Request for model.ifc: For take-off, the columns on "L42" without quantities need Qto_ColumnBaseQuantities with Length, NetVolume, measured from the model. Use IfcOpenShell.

First a look at what the model holds.

```python
import ifcopenshell
import ifcopenshell.util.element
import ifcopenshell.util.unit

model = ifcopenshell.open("model.ifc")
print(model.schema)
for unit_type in ("LENGTHUNIT", "AREAUNIT", "VOLUMEUNIT"):
    print(unit_type, ifcopenshell.util.unit.calculate_unit_scale(model, unit_type))
storey = next(s for s in model.by_type("IfcBuildingStorey") if s.Name == "L42")
columns = [e for e in ifcopenshell.util.element.get_decomposition(storey) if e.is_a("IfcColumn")]
for e in sorted(columns, key=lambda e: e.id()):
    print(e.id(), e.is_a(), e.Name, list(ifcopenshell.util.element.get_psets(e, qtos_only=True)), sep=" | ")
```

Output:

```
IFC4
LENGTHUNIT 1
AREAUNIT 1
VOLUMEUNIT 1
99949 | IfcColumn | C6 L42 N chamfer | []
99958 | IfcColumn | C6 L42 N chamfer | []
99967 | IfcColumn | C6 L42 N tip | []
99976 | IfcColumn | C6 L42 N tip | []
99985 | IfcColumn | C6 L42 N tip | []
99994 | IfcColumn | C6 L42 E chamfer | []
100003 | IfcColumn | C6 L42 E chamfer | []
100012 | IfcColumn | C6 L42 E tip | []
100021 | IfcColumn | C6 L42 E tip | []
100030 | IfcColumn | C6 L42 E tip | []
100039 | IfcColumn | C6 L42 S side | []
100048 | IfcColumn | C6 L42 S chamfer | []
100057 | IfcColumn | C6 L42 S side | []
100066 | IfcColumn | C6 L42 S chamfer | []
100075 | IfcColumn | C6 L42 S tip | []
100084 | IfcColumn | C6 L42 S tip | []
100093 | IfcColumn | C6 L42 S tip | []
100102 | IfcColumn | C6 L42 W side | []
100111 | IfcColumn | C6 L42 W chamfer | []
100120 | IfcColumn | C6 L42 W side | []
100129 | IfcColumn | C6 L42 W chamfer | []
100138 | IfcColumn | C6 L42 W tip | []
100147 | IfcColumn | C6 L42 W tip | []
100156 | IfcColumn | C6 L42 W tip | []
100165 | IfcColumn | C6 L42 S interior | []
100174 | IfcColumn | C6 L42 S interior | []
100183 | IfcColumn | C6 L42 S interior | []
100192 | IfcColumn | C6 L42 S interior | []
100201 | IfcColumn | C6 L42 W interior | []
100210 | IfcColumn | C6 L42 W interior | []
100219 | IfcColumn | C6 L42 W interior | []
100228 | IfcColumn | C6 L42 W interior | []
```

```python
import ifcopenshell
import ifcopenshell.api.pset
import ifcopenshell.geom
import ifcopenshell.util.element
import ifcopenshell.util.shape
import ifcopenshell.util.unit

model = ifcopenshell.open("model.ifc")
unit_scale = ifcopenshell.util.unit.calculate_unit_scale(model)
volume_scale = ifcopenshell.util.unit.calculate_unit_scale(model, "VOLUMEUNIT")
settings = ifcopenshell.geom.settings()

storey = next(s for s in model.by_type("IfcBuildingStorey") if s.Name == "L42")
columns = [e for e in ifcopenshell.util.element.get_decomposition(storey) if e.is_a("IfcColumn")]

for e in sorted(columns, key=lambda e: e.id()):
    if ifcopenshell.util.element.get_psets(e, qtos_only=True, should_inherit=False):
        continue
    # Geometry comes back in metres, in the element's own axes.
    shape = ifcopenshell.geom.create_shape(settings, e)
    values = {
        "Length": ifcopenshell.util.shape.get_z(shape.geometry) / unit_scale,
        "NetVolume": ifcopenshell.util.shape.get_volume(shape.geometry) / volume_scale,
    }
    qto = ifcopenshell.api.pset.add_qto(model, product=e, name="Qto_ColumnBaseQuantities")
    ifcopenshell.api.pset.edit_qto(model, qto=qto, properties=values)
    print(e.id(), {k: round(v, 3) for k, v in values.items()})

model.write("model_updated.ifc")
```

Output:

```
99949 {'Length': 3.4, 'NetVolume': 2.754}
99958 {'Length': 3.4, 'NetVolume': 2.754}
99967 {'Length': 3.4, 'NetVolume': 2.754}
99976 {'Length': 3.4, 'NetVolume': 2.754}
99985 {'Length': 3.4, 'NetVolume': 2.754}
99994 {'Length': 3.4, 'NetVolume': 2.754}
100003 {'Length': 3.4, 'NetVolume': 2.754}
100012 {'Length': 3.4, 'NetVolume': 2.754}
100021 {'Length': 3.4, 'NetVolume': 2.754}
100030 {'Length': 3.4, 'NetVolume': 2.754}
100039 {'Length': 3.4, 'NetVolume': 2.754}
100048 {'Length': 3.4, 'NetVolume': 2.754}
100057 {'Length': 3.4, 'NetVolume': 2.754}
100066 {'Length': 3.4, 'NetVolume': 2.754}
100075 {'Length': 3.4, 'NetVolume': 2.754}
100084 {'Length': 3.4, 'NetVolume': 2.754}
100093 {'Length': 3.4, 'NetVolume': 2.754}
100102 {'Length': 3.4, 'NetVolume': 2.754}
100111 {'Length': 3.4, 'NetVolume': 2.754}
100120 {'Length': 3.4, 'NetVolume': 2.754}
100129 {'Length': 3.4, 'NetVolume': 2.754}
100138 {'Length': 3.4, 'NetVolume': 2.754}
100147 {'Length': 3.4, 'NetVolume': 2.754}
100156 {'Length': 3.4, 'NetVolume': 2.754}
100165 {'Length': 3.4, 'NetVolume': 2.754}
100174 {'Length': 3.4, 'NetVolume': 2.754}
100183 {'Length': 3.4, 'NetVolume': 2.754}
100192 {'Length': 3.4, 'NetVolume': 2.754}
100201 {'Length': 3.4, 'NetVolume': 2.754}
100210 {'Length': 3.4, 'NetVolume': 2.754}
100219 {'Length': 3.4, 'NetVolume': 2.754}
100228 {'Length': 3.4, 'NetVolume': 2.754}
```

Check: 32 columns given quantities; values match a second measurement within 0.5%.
